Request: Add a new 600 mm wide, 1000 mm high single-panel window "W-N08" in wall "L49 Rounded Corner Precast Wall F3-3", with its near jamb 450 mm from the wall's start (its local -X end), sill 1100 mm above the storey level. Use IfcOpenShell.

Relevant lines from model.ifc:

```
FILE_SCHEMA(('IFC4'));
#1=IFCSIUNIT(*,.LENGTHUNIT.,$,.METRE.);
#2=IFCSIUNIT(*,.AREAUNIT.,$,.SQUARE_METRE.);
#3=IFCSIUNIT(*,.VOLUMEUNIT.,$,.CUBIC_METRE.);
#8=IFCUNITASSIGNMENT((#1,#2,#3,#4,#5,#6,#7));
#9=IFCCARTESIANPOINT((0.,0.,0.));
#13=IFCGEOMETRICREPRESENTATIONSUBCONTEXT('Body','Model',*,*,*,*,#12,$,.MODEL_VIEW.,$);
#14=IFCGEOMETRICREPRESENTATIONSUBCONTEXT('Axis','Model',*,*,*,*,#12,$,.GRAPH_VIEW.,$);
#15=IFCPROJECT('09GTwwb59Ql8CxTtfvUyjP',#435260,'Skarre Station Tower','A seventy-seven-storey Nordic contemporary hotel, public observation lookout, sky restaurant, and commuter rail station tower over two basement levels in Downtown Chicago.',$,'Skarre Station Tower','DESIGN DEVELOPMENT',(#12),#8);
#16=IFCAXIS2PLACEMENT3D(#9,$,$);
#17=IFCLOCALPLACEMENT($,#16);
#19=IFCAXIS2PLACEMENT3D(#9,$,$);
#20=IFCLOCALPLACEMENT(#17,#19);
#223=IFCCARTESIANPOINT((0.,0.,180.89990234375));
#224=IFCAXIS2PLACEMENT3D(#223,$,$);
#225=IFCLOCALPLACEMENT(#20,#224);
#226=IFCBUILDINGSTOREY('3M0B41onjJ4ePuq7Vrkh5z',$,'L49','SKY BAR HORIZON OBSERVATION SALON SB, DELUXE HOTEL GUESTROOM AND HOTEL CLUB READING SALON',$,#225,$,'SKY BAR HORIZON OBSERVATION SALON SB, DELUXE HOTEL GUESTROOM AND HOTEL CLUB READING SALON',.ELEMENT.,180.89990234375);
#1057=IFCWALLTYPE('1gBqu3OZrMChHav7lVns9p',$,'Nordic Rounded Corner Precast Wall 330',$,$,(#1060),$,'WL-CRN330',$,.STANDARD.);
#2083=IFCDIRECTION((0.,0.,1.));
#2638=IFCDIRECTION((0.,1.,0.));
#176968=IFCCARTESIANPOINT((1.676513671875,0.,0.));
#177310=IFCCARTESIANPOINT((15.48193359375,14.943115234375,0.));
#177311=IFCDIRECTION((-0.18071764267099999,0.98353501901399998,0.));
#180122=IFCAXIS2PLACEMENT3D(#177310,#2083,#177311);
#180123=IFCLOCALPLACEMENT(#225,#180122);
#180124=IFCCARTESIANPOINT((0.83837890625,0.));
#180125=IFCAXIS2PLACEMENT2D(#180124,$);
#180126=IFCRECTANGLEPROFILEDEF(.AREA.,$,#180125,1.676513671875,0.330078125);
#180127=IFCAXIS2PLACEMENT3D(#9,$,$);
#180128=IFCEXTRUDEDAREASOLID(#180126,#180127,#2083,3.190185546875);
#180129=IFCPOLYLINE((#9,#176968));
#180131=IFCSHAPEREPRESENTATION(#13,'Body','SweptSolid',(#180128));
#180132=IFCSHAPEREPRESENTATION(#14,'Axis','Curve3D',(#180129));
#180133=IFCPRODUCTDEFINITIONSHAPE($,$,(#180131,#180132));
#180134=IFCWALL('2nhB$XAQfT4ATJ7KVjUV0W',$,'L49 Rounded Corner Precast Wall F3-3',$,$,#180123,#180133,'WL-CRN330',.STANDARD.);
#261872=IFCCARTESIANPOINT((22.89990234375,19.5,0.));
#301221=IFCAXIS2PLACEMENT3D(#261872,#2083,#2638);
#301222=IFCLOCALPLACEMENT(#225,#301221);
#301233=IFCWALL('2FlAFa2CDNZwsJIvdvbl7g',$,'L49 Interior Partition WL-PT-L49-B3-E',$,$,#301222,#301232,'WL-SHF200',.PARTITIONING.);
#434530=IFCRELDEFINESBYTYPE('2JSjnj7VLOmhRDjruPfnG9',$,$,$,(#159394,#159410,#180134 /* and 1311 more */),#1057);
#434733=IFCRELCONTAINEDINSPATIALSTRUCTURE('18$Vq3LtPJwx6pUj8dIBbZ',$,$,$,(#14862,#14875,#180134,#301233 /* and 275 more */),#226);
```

```python
import numpy as np
import ifcopenshell
import ifcopenshell.api.feature
import ifcopenshell.api.geometry
import ifcopenshell.api.root
import ifcopenshell.api.spatial
import ifcopenshell.geom
import ifcopenshell.util.element
import ifcopenshell.util.placement
import ifcopenshell.util.representation
import ifcopenshell.util.shape
import ifcopenshell.util.unit

model = ifcopenshell.open("model.ifc")
unit_scale = ifcopenshell.util.unit.calculate_unit_scale(model)
settings = ifcopenshell.geom.settings()


def volume(element):
    """Net volume in cubic metres, openings subtracted."""
    shape = ifcopenshell.geom.create_shape(settings, element)
    return ifcopenshell.util.shape.get_volume(shape.geometry)


wall = model.by_id(180134)
storey = ifcopenshell.util.element.get_container(wall, ifc_class="IfcBuildingStorey")
context = ifcopenshell.util.representation.get_context(model, "Model", "Body", "MODEL_VIEW")
before = volume(wall)

width, height, from_end, sill = 0.6, 1, 0.45, 1.1  # metres

# The wall runs along its own X axis, and the end named is its -X end.
wall_shape = ifcopenshell.geom.create_shape(settings, wall)
x, y, z = ifcopenshell.util.shape.get_vertices(wall_shape.geometry).T
start = x.min() + from_end
face, thickness = float(y.min()), float(y.max() - y.min())
wall_matrix = ifcopenshell.util.placement.get_local_placement(wall.ObjectPlacement)
level = ifcopenshell.util.placement.get_local_placement(storey.ObjectPlacement)[2, 3]


def in_wall(x, y):
    """Placement at x, y metres in the wall's axes, at sill height."""
    matrix = wall_matrix.copy()
    matrix[:, 3] = wall_matrix @ np.array([x / unit_scale, y / unit_scale, 0.0, 1.0])
    matrix[2, 3] = level + sill / unit_scale
    return matrix


# Opening: a box that overshoots both wall faces by 50 mm.
opening = ifcopenshell.api.root.create_entity(model, ifc_class="IfcOpeningElement", predefined_type="OPENING")
box = ifcopenshell.api.geometry.add_wall_representation(
    model, context=context, length=width, height=height, thickness=thickness + 0.1
)
ifcopenshell.api.geometry.assign_representation(model, product=opening, representation=box)
ifcopenshell.api.geometry.edit_object_placement(model, product=opening, matrix=in_wall(start, face - 0.05), is_si=False)
ifcopenshell.api.feature.add_feature(model, feature=opening, element=wall)

window = ifcopenshell.api.root.create_entity(model, ifc_class="IfcWindow", name="W-N08", predefined_type="WINDOW")
window.OverallWidth, window.OverallHeight = width / unit_scale, height / unit_scale
window.PartitioningType = "SINGLE_PANEL"
body = ifcopenshell.api.geometry.add_window_representation(
    model,
    context=context,
    overall_width=window.OverallWidth,
    overall_height=window.OverallHeight,
    partition_type="SINGLE_PANEL",
)
ifcopenshell.api.geometry.assign_representation(model, product=window, representation=body)
ifcopenshell.api.spatial.assign_container(model, products=[window], relating_structure=storey)
ifcopenshell.api.feature.add_filling(model, opening=opening, element=window)

# Centre the window in the wall's thickness.
ifcopenshell.api.geometry.edit_object_placement(model, product=window, matrix=in_wall(start, face), is_si=False)
window_shape = ifcopenshell.geom.create_shape(settings, window)
depth = ifcopenshell.util.shape.get_vertices(window_shape.geometry)[:, 1]
offset = face + thickness / 2 - (depth.min() + depth.max()) / 2
ifcopenshell.api.geometry.edit_object_placement(model, product=window, matrix=in_wall(start, offset), is_si=False)

after = volume(wall)

print(f"wall volume {before:.3f} -> {after:.3f} m3")

model.write("model_edited.ifc")
```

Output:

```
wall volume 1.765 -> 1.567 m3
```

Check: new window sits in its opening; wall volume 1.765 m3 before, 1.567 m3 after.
